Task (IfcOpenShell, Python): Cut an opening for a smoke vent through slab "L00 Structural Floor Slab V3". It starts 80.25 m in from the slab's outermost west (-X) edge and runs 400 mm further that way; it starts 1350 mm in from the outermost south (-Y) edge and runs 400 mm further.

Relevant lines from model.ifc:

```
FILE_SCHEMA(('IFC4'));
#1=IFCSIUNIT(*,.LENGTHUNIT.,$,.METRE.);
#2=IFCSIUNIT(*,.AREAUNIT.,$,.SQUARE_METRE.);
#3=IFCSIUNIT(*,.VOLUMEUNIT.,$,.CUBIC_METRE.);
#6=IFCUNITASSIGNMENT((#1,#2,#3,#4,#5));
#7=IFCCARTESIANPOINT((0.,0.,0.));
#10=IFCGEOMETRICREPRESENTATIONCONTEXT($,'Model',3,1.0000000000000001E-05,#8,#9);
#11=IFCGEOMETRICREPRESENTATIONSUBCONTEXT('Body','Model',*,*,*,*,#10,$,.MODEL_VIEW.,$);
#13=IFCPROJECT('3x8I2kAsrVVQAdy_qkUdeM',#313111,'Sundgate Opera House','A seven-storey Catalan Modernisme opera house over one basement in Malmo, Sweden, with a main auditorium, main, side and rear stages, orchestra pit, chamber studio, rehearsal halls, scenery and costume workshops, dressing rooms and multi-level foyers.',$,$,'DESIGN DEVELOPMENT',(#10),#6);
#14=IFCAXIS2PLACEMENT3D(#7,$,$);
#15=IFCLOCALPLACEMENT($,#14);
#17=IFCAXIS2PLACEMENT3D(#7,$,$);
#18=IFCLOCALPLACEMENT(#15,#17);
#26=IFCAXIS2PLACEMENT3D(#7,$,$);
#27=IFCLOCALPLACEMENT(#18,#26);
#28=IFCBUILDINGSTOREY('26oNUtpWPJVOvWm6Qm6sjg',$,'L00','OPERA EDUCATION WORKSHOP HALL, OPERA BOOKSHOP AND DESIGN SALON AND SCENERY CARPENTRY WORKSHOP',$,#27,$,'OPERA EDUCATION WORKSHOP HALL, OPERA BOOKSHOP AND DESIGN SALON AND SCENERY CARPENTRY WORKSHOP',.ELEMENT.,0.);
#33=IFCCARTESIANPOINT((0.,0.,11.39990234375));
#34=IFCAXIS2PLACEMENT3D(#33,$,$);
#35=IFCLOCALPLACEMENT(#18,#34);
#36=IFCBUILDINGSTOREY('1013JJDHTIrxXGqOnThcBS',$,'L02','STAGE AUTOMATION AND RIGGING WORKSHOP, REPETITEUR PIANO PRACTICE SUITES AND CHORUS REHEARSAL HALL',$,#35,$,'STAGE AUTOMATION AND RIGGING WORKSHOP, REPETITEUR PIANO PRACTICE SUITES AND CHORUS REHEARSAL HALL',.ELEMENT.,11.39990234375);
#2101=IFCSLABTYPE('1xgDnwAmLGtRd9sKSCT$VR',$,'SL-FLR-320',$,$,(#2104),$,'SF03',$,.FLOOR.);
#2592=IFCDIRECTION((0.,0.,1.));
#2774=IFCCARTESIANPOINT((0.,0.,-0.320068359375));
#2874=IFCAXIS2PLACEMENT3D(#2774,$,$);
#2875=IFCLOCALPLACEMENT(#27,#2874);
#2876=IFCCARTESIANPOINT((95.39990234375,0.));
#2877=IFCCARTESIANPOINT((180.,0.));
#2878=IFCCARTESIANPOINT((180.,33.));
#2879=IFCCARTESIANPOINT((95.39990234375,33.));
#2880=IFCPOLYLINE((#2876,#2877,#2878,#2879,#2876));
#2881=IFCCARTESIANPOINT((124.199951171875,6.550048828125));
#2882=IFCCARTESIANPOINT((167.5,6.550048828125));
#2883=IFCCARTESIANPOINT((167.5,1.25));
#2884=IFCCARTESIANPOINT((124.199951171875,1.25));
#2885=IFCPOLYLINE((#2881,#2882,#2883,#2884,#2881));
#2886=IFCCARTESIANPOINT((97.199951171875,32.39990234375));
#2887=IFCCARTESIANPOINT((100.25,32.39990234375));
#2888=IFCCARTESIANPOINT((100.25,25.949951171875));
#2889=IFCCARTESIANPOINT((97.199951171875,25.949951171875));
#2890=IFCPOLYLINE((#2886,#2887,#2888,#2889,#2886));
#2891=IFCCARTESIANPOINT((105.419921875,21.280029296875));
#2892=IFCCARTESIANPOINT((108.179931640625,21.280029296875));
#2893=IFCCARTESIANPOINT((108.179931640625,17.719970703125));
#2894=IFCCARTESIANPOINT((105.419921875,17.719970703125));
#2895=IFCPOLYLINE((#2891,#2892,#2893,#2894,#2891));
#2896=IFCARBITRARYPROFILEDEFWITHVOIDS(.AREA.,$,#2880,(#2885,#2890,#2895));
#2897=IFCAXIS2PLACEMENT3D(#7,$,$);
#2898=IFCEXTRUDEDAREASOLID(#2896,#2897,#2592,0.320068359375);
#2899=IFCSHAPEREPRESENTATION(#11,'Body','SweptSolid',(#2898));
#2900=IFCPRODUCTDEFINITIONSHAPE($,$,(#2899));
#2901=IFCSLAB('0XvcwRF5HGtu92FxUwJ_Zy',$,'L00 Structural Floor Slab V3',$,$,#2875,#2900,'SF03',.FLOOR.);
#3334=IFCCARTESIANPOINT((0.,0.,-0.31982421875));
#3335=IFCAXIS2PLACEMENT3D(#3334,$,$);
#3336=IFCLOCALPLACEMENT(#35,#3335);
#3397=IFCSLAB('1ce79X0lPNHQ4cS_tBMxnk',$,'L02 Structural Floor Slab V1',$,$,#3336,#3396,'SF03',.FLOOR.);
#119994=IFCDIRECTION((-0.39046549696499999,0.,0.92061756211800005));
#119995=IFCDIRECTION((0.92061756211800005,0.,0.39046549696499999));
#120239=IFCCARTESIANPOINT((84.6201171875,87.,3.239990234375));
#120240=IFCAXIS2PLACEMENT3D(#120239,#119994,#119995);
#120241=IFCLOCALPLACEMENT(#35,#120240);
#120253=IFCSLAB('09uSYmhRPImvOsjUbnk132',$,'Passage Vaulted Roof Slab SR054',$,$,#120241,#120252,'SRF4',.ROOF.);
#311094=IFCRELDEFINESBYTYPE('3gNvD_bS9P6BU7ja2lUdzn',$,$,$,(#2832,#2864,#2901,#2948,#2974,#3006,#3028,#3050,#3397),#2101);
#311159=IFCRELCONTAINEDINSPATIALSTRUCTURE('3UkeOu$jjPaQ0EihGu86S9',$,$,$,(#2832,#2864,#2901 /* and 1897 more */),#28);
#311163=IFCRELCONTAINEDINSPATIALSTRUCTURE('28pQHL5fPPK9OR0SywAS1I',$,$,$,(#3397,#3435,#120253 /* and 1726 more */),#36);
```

```python
import numpy as np
import ifcopenshell
import ifcopenshell.api.feature
import ifcopenshell.api.geometry
import ifcopenshell.api.root
import ifcopenshell.geom
import ifcopenshell.util.placement
import ifcopenshell.util.representation
import ifcopenshell.util.shape
import ifcopenshell.util.unit

model = ifcopenshell.open("model.ifc")
unit_scale = ifcopenshell.util.unit.calculate_unit_scale(model)
settings = ifcopenshell.geom.settings()


def volume(element):
    """Net volume in cubic metres, openings subtracted."""
    shape = ifcopenshell.geom.create_shape(settings, element)
    return ifcopenshell.util.shape.get_volume(shape.geometry)


slab = model.by_guid("0XvcwRF5HGtu92FxUwJ_Zy")
before = volume(slab)

# Extent in the slab's own axes, in metres. The edges named are its -X and -Y sides.
slab_shape = ifcopenshell.geom.create_shape(settings, slab)
vertices = ifcopenshell.util.shape.get_vertices(slab_shape.geometry)
x_min, y_min, bottom = vertices.min(axis=0)
top = vertices[:, 2].max()

opening = ifcopenshell.api.root.create_entity(model, ifc_class="IfcOpeningElement", name="Smoke vent opening", predefined_type="OPENING")
context = ifcopenshell.util.representation.get_context(model, "Model", "Body", "MODEL_VIEW")
width, depth = 0.4, 0.4
outline = [(0.0, 0.0), (width, 0.0), (width, depth), (0.0, depth), (0.0, 0.0)]
# Overshoot both faces by 50 mm so the cut is clean.
shape = ifcopenshell.api.geometry.add_slab_representation(
    model, context=context, depth=top - bottom + 0.1, polyline=outline
)
ifcopenshell.api.geometry.assign_representation(model, product=opening, representation=shape)

matrix = ifcopenshell.util.placement.get_local_placement(slab.ObjectPlacement)
matrix[:, 3] = matrix @ np.append(np.array([x_min + 80.25, y_min + 1.35, bottom - 0.05]) / unit_scale, 1.0)
ifcopenshell.api.geometry.edit_object_placement(model, product=opening, matrix=matrix, is_si=False)
ifcopenshell.api.feature.add_feature(model, feature=opening, element=slab)

after = volume(slab)

print(f"slab volume {before:.3f} -> {after:.3f} m3")

model.write("model_v2.ifc")
```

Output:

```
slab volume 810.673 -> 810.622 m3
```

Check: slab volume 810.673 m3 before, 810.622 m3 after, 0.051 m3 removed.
